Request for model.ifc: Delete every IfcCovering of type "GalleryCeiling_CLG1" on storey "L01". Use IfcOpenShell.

First a look at what the model holds.

```python
import ifcopenshell
import ifcopenshell.util.element

model = ifcopenshell.open("model.ifc")
print(model.schema)
storey = next(s for s in model.by_type("IfcBuildingStorey") if s.Name == "L01")
coverings = [e for e in ifcopenshell.util.element.get_decomposition(storey) if e.is_a("IfcCovering")]
seen = {}
for e in coverings:
    element_type = ifcopenshell.util.element.get_type(e)
    name = element_type.Name if element_type not in (None, e) else None
    seen[name] = seen.get(name, 0) + 1
for name, count in sorted(seen.items(), key=str):
    print(count, "x", name)
```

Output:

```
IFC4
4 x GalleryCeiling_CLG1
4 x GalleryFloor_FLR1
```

```python
import ifcopenshell
import ifcopenshell.api.root
import ifcopenshell.util.element

model = ifcopenshell.open("model.ifc")

storey = next(s for s in model.by_type("IfcBuildingStorey") if s.Name == "L01")
coverings = [e for e in ifcopenshell.util.element.get_decomposition(storey) if e.is_a("IfcCovering")]
targets = [e for e in coverings if (t := ifcopenshell.util.element.get_type(e)) not in (None, e) and t.Name == "GalleryCeiling_CLG1"]

for e in targets:
    ifcopenshell.api.root.remove_product(model, product=e)
print(len(targets), "removed")

model.write("model_rev.ifc")
```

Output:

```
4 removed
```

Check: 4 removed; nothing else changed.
